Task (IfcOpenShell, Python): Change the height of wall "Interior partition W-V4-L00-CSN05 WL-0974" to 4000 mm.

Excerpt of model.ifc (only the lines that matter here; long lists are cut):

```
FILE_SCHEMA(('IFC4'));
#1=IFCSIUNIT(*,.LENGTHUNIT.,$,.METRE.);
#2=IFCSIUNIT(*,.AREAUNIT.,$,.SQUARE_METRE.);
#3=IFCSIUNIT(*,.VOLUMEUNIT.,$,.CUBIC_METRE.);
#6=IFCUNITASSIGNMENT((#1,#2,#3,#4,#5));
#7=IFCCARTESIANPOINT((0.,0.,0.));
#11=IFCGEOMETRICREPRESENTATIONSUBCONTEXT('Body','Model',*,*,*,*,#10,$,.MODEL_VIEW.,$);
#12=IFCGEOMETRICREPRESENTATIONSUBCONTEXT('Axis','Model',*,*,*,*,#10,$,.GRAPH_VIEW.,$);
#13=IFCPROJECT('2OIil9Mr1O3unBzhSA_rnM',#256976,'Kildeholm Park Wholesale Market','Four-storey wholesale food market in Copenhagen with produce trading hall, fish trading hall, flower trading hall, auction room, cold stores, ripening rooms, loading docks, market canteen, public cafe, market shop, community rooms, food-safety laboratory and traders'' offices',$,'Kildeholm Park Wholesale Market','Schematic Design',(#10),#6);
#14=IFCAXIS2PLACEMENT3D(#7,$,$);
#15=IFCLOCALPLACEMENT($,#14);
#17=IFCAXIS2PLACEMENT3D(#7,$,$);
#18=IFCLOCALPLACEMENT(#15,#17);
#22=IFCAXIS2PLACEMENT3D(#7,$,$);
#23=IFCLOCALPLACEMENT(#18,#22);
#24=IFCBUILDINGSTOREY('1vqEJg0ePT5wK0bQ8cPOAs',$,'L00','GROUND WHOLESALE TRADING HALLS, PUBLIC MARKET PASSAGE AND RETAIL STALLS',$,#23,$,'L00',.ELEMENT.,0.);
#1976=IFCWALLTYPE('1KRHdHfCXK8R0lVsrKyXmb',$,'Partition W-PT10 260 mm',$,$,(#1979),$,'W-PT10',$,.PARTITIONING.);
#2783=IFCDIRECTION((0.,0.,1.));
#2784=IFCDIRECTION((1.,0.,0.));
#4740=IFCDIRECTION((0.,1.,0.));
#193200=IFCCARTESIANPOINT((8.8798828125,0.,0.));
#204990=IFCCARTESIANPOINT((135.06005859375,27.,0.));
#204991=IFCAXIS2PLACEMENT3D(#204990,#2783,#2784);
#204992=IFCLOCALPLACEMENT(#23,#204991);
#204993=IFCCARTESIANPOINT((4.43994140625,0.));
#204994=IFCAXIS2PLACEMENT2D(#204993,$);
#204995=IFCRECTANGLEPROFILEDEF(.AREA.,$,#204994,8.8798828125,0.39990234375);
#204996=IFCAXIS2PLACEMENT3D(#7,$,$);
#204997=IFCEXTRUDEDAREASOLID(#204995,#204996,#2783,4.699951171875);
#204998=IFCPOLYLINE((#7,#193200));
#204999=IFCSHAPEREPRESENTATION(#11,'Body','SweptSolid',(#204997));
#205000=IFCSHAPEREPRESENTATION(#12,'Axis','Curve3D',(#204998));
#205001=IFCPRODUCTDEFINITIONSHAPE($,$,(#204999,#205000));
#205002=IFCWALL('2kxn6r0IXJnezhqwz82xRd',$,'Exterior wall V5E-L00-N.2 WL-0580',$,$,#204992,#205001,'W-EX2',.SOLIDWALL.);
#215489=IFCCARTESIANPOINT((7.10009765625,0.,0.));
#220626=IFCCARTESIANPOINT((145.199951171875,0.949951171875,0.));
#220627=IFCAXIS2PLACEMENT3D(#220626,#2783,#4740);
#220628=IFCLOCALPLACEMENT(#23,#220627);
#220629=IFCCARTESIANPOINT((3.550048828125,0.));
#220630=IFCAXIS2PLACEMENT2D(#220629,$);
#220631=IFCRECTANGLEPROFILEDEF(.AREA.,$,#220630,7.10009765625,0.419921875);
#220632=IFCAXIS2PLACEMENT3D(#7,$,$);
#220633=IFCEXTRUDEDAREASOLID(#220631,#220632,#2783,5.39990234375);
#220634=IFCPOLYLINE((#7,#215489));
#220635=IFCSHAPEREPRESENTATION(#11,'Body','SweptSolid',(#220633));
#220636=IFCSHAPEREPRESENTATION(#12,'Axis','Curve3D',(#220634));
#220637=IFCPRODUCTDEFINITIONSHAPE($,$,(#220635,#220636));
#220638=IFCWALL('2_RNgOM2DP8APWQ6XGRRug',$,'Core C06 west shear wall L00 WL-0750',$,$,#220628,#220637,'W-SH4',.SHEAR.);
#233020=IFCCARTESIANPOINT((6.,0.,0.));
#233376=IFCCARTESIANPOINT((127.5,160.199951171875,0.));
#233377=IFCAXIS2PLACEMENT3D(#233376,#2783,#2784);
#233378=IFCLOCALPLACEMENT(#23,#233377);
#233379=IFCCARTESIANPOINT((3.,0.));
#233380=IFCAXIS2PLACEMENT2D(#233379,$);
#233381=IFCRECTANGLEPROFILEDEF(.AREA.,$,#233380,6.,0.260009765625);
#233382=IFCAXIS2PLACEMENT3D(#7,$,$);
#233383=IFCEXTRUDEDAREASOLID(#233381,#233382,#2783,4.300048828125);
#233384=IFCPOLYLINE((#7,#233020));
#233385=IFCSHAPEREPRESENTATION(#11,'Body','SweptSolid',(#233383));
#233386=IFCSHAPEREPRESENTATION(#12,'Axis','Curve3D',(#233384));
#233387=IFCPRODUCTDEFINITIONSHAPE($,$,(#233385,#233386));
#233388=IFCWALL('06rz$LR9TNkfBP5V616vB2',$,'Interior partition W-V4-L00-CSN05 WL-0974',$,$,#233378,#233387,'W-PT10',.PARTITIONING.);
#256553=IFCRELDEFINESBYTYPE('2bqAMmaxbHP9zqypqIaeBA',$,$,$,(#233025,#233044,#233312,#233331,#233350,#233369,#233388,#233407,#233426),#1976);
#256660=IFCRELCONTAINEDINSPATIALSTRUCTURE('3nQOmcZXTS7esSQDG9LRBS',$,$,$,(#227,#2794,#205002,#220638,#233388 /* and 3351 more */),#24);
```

```python
import ifcopenshell
import ifcopenshell.geom
import ifcopenshell.util.representation
import ifcopenshell.util.shape

model = ifcopenshell.open("model.ifc")
settings = ifcopenshell.geom.settings()


def volume(element):
    """Net volume in cubic metres, openings subtracted."""
    shape = ifcopenshell.geom.create_shape(settings, element)
    return ifcopenshell.util.shape.get_volume(shape.geometry)


wall = model.by_guid("06rz$LR9TNkfBP5V616vB2")
before = volume(wall)

body = ifcopenshell.util.representation.get_representation(wall, "Model", "Body")
solid = body.Items[0]
old_height = solid.Depth
solid.Depth = 4.0
after = volume(wall)

print(f"height {old_height:g} -> {solid.Depth:g}, volume {before:.3f} -> {after:.3f} m3")

model.write("model_edited.ifc")
```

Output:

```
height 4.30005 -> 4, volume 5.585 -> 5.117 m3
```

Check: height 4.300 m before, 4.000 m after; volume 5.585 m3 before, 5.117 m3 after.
